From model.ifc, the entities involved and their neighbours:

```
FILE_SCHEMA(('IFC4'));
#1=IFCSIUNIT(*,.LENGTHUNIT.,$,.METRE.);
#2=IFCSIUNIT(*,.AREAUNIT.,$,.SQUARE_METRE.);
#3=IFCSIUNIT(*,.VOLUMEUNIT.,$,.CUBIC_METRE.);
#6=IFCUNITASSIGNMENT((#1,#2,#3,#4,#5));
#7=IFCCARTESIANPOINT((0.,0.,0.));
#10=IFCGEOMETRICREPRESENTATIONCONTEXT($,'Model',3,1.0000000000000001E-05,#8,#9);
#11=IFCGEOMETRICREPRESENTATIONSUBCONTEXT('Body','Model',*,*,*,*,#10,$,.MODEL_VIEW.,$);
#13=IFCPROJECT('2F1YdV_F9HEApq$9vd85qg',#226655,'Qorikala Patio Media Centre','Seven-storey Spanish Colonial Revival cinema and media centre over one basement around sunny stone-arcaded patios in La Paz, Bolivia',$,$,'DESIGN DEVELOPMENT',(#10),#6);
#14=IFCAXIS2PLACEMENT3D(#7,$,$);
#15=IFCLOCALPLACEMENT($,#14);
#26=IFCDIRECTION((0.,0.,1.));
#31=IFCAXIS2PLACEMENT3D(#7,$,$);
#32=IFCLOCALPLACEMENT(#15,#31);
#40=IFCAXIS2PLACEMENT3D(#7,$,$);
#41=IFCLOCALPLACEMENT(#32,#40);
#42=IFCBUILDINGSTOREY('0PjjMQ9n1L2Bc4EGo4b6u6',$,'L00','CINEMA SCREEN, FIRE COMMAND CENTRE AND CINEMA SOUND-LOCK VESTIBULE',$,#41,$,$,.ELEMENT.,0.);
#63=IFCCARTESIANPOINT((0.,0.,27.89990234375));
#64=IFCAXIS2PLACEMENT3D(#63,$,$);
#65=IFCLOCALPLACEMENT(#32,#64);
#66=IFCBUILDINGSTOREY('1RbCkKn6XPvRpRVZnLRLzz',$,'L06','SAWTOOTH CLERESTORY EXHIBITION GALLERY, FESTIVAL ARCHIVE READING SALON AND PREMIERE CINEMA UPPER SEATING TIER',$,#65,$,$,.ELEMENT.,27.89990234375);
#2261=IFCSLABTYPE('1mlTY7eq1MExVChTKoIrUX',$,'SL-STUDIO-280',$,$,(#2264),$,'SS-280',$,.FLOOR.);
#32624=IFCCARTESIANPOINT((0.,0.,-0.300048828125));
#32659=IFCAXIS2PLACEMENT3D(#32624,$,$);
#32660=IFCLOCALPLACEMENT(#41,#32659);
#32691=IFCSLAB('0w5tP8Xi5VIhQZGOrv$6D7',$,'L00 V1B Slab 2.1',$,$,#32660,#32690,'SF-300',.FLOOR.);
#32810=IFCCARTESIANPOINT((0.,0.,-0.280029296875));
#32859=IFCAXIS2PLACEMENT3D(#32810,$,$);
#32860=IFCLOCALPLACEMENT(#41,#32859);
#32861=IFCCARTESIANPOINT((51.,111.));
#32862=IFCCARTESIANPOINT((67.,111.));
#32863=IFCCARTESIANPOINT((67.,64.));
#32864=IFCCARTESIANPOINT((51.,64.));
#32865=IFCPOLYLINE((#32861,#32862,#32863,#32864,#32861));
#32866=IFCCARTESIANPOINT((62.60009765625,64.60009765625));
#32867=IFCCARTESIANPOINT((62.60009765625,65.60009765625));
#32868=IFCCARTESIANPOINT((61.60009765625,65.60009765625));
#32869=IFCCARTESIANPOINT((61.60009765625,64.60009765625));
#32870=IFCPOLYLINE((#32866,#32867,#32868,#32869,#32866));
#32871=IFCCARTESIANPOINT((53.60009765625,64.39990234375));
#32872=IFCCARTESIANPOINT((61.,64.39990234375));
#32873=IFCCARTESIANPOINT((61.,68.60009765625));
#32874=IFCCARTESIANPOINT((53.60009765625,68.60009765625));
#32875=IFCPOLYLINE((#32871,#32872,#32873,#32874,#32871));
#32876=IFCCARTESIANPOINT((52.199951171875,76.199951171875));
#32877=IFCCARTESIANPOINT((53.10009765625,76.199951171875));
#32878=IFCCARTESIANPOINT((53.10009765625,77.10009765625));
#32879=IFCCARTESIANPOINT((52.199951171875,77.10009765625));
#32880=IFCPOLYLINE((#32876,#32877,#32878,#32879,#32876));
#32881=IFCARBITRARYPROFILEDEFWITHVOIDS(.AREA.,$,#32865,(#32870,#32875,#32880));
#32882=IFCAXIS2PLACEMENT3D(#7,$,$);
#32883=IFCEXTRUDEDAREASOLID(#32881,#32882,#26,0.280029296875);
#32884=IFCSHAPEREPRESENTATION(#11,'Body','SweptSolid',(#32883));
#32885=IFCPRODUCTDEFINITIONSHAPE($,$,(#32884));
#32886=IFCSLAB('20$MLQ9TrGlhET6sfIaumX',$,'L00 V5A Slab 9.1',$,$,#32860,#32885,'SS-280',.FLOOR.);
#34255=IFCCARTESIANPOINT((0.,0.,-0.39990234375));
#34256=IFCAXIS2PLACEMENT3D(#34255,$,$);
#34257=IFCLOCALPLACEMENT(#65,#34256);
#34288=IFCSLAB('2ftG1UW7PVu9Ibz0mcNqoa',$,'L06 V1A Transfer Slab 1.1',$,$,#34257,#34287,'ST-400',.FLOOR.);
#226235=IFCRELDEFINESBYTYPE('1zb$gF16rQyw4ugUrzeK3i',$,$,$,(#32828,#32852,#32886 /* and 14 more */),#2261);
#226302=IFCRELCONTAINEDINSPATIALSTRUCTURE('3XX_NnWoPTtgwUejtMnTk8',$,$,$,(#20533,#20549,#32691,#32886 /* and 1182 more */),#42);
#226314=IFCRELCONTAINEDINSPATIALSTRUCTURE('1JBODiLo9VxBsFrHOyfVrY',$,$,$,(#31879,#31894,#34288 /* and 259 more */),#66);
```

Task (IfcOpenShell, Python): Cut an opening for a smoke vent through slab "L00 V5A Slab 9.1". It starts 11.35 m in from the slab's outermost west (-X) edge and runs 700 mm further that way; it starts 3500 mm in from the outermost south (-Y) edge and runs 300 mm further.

```python
import numpy as np
import ifcopenshell
import ifcopenshell.api.feature
import ifcopenshell.api.geometry
import ifcopenshell.api.root
import ifcopenshell.geom
import ifcopenshell.util.placement
import ifcopenshell.util.representation
import ifcopenshell.util.shape
import ifcopenshell.util.unit

model = ifcopenshell.open("model.ifc")
unit_scale = ifcopenshell.util.unit.calculate_unit_scale(model)
settings = ifcopenshell.geom.settings()


def volume(element):
    """Net volume in cubic metres, openings subtracted."""
    shape = ifcopenshell.geom.create_shape(settings, element)
    return ifcopenshell.util.shape.get_volume(shape.geometry)


slab = model.by_guid("20$MLQ9TrGlhET6sfIaumX")
before = volume(slab)

# Extent in the slab's own axes, in metres. The edges named are its -X and -Y sides.
slab_shape = ifcopenshell.geom.create_shape(settings, slab)
vertices = ifcopenshell.util.shape.get_vertices(slab_shape.geometry)
x_min, y_min, bottom = vertices.min(axis=0)
top = vertices[:, 2].max()

opening = ifcopenshell.api.root.create_entity(model, ifc_class="IfcOpeningElement", name="Smoke vent opening", predefined_type="OPENING")
context = ifcopenshell.util.representation.get_context(model, "Model", "Body", "MODEL_VIEW")
width, depth = 0.7, 0.3
outline = [(0.0, 0.0), (width, 0.0), (width, depth), (0.0, depth), (0.0, 0.0)]
# Overshoot both faces by 50 mm so the cut is clean.
shape = ifcopenshell.api.geometry.add_slab_representation(
    model, context=context, depth=top - bottom + 0.1, polyline=outline
)
ifcopenshell.api.geometry.assign_representation(model, product=opening, representation=shape)

matrix = ifcopenshell.util.placement.get_local_placement(slab.ObjectPlacement)
matrix[:, 3] = matrix @ np.append(np.array([x_min + 11.35, y_min + 3.5, bottom - 0.05]) / unit_scale, 1.0)
ifcopenshell.api.geometry.edit_object_placement(model, product=opening, matrix=matrix, is_si=False)
ifcopenshell.api.feature.add_feature(model, feature=opening, element=slab)

after = volume(slab)

print(f"slab volume {before:.3f} -> {after:.3f} m3")

model.write("model-out.ifc")
```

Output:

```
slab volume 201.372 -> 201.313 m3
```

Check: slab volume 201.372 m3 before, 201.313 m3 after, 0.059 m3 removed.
